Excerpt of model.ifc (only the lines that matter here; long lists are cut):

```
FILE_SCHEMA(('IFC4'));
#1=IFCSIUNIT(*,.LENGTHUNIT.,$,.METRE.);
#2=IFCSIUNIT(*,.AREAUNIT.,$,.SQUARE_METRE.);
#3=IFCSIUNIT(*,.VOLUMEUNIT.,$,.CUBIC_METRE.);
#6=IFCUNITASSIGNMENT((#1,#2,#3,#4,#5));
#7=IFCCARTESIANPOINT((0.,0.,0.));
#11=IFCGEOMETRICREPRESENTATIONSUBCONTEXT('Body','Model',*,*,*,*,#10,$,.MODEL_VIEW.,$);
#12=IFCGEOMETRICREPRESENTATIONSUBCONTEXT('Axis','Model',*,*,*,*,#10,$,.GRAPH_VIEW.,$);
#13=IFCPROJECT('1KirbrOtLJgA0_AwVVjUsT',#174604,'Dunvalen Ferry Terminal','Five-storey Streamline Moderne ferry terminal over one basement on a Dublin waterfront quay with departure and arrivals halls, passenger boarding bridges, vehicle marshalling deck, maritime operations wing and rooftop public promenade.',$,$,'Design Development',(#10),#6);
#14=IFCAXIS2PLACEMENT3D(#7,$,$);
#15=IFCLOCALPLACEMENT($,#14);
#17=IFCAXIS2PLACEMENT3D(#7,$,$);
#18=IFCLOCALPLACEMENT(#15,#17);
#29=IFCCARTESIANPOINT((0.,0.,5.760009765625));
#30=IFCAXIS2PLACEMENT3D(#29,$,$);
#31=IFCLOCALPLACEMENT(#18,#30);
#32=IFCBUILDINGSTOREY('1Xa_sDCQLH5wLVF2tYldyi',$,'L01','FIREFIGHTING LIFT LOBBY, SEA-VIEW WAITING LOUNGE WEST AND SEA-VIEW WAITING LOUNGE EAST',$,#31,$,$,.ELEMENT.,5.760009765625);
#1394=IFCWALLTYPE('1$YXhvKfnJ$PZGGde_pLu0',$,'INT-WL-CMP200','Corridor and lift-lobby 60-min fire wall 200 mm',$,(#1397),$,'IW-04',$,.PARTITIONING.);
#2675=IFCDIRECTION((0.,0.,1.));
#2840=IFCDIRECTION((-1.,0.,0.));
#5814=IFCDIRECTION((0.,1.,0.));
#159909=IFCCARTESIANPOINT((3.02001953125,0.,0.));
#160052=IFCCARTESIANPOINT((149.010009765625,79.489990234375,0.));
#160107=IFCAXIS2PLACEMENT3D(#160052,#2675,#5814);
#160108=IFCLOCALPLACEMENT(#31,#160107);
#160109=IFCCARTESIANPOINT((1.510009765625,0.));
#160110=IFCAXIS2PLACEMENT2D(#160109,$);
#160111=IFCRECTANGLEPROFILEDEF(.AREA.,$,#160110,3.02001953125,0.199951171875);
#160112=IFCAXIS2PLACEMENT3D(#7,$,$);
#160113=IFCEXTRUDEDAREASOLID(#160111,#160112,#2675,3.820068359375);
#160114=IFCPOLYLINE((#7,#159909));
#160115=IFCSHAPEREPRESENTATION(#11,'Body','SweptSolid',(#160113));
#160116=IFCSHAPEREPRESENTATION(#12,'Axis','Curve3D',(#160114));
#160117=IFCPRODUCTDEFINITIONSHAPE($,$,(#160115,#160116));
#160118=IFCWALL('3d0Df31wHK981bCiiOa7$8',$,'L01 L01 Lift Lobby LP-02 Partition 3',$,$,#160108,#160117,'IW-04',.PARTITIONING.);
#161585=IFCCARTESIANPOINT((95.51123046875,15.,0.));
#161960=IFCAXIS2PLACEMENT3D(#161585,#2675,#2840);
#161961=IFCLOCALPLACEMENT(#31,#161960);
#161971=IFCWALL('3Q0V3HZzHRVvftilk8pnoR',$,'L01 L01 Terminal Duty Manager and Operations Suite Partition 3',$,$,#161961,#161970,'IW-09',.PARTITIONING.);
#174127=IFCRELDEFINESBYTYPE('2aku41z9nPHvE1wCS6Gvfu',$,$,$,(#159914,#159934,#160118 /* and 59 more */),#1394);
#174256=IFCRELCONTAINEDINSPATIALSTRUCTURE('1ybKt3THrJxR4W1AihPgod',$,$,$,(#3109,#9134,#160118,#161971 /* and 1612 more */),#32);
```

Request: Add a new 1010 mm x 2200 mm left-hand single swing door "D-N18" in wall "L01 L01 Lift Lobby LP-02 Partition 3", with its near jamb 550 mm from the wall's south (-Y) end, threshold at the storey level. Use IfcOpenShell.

```python
import numpy as np
import ifcopenshell
import ifcopenshell.api.feature
import ifcopenshell.api.geometry
import ifcopenshell.api.root
import ifcopenshell.api.spatial
import ifcopenshell.geom
import ifcopenshell.util.element
import ifcopenshell.util.placement
import ifcopenshell.util.representation
import ifcopenshell.util.shape
import ifcopenshell.util.unit

model = ifcopenshell.open("model.ifc")
unit_scale = ifcopenshell.util.unit.calculate_unit_scale(model)
settings = ifcopenshell.geom.settings()


def volume(element):
    """Net volume in cubic metres, openings subtracted."""
    shape = ifcopenshell.geom.create_shape(settings, element)
    return ifcopenshell.util.shape.get_volume(shape.geometry)


wall = model.by_guid("3d0Df31wHK981bCiiOa7$8")
storey = ifcopenshell.util.element.get_container(wall, ifc_class="IfcBuildingStorey")
context = ifcopenshell.util.representation.get_context(model, "Model", "Body", "MODEL_VIEW")
before = volume(wall)

width, height, from_end, sill = 1.01, 2.2, 0.55, 0.0  # metres

# The wall runs along its own X axis, and the end named is its -X end.
wall_shape = ifcopenshell.geom.create_shape(settings, wall)
x, y, z = ifcopenshell.util.shape.get_vertices(wall_shape.geometry).T
start = x.min() + from_end
face, thickness = float(y.min()), float(y.max() - y.min())
wall_matrix = ifcopenshell.util.placement.get_local_placement(wall.ObjectPlacement)
level = ifcopenshell.util.placement.get_local_placement(storey.ObjectPlacement)[2, 3]


def in_wall(x, y):
    """Placement at x, y metres in the wall's axes, at sill height."""
    matrix = wall_matrix.copy()
    matrix[:, 3] = wall_matrix @ np.array([x / unit_scale, y / unit_scale, 0.0, 1.0])
    matrix[2, 3] = level + sill / unit_scale
    return matrix


# Opening: a box that overshoots both wall faces by 50 mm.
opening = ifcopenshell.api.root.create_entity(model, ifc_class="IfcOpeningElement", predefined_type="OPENING")
box = ifcopenshell.api.geometry.add_wall_representation(
    model, context=context, length=width, height=height, thickness=thickness + 0.1
)
ifcopenshell.api.geometry.assign_representation(model, product=opening, representation=box)
ifcopenshell.api.geometry.edit_object_placement(model, product=opening, matrix=in_wall(start, face - 0.05), is_si=False)
ifcopenshell.api.feature.add_feature(model, feature=opening, element=wall)

door = ifcopenshell.api.root.create_entity(model, ifc_class="IfcDoor", name="D-N18", predefined_type="DOOR")
door.OverallWidth, door.OverallHeight = width / unit_scale, height / unit_scale
door.OperationType = "SINGLE_SWING_LEFT"
body = ifcopenshell.api.geometry.add_door_representation(
    model,
    context=context,
    overall_width=door.OverallWidth,
    overall_height=door.OverallHeight,
    operation_type="SINGLE_SWING_LEFT",
    lining_properties={"LiningDepth": thickness / unit_scale, "ThresholdDepth": thickness / unit_scale},
)
ifcopenshell.api.geometry.assign_representation(model, product=door, representation=body)
ifcopenshell.api.spatial.assign_container(model, products=[door], relating_structure=storey)
ifcopenshell.api.feature.add_filling(model, opening=opening, element=door)

# The lining spans the wall, so the door starts at the wall face.
ifcopenshell.api.geometry.edit_object_placement(model, product=door, matrix=in_wall(start, face), is_si=False)

after = volume(wall)

print(f"wall volume {before:.3f} -> {after:.3f} m3")

model.write("model_rev.ifc")
```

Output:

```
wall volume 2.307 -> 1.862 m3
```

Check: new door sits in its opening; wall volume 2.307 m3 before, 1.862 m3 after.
